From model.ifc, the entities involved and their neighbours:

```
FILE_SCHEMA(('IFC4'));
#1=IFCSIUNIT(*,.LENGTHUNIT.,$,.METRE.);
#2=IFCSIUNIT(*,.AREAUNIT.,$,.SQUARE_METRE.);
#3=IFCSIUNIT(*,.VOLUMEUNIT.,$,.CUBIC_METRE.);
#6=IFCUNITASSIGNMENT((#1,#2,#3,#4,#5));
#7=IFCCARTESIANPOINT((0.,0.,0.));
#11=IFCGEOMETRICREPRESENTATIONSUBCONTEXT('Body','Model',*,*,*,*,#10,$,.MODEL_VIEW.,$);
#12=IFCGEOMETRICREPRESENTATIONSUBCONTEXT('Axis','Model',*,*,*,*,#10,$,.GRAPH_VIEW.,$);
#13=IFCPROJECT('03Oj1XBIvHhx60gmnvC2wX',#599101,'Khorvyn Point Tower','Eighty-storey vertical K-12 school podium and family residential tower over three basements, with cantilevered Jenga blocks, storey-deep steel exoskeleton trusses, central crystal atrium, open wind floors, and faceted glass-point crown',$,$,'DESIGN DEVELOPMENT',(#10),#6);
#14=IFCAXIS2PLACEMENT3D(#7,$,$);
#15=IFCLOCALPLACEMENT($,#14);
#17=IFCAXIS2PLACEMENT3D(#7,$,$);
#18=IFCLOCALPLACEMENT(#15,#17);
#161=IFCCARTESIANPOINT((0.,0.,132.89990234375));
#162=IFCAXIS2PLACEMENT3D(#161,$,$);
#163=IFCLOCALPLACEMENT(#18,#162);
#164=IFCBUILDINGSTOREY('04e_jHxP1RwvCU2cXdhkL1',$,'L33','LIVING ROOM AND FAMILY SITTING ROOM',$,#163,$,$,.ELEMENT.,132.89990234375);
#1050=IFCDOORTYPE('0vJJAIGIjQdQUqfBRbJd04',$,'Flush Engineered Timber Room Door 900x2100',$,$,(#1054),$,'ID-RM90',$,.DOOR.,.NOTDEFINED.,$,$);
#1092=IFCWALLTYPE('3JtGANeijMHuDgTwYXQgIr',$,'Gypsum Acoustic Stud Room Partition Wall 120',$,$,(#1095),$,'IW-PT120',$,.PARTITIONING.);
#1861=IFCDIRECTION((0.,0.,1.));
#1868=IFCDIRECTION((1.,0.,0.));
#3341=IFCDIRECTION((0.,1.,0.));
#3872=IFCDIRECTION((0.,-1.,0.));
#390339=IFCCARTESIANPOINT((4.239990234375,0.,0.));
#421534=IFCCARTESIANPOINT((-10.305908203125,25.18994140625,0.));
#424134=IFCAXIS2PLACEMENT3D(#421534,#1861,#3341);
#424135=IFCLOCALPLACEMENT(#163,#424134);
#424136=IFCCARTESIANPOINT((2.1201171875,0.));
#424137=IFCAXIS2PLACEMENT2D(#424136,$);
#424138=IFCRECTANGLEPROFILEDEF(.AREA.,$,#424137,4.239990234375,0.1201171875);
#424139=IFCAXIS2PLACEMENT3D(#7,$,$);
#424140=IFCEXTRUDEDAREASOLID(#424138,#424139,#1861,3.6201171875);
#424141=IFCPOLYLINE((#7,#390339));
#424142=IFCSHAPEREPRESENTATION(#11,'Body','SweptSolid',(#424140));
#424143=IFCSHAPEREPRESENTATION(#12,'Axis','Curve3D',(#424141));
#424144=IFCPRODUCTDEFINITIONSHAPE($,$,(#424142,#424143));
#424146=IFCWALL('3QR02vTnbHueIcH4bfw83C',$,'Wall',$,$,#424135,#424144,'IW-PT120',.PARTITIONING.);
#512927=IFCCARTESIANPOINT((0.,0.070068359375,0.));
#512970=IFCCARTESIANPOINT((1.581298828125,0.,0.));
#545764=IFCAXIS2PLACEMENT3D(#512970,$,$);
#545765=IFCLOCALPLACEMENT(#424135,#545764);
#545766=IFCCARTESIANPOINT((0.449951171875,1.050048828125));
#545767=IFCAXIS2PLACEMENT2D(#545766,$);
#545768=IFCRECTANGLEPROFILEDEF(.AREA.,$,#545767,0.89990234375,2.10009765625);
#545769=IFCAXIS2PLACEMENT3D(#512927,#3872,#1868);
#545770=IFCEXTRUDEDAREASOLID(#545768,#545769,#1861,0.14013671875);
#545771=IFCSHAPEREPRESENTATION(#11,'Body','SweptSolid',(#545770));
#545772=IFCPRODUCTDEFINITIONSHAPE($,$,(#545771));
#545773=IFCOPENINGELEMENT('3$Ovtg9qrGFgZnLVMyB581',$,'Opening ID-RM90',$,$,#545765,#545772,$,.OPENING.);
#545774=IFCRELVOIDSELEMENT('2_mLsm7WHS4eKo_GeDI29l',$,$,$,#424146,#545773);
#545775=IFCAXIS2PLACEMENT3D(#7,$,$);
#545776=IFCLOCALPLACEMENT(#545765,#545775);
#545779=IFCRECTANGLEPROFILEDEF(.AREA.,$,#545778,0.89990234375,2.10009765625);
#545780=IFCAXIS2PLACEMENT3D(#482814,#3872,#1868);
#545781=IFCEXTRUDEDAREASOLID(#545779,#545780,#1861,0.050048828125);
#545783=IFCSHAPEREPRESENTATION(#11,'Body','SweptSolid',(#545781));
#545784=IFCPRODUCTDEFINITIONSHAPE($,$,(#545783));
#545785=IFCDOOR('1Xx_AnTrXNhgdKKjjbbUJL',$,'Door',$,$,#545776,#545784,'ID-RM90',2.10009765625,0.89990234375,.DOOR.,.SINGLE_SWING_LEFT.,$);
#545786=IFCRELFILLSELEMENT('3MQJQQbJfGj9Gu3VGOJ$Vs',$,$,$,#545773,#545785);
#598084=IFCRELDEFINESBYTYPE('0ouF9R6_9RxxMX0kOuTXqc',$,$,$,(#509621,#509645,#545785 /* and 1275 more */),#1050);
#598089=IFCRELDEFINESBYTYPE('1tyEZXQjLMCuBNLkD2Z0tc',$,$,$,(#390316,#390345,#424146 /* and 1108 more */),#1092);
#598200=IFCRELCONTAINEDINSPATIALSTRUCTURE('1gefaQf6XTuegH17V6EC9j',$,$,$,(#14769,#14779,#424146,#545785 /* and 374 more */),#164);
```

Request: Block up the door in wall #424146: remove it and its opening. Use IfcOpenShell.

```python
import ifcopenshell
import ifcopenshell.api.feature
import ifcopenshell.api.root
import ifcopenshell.geom
import ifcopenshell.util.shape

model = ifcopenshell.open("model.ifc")
settings = ifcopenshell.geom.settings()


def volume(element):
    """Net volume in cubic metres, openings subtracted."""
    shape = ifcopenshell.geom.create_shape(settings, element)
    return ifcopenshell.util.shape.get_volume(shape.geometry)


door = model.by_guid("1Xx_AnTrXNhgdKKjjbbUJL")
opening = door.FillsVoids[0].RelatingOpeningElement
wall = opening.VoidsElements[0].RelatingBuildingElement
before = volume(wall)

ifcopenshell.api.root.remove_product(model, product=door)
ifcopenshell.api.feature.remove_feature(model, feature=opening)

after = volume(wall)

print(f"wall volume {before:.3f} -> {after:.3f} m3")

model.write("model_v2.ifc")
```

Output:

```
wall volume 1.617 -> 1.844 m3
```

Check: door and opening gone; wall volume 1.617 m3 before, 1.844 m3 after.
